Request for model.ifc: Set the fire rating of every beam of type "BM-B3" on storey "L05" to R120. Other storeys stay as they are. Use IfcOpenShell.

First a look at what the model holds.

```python
import ifcopenshell
import ifcopenshell.util.element

model = ifcopenshell.open("model.ifc")
print(model.schema)
storey = next(s for s in model.by_type("IfcBuildingStorey") if s.Name == "L05")
beams = [e for e in ifcopenshell.util.element.get_decomposition(storey) if e.is_a("IfcBeam")]
seen = {}
for e in beams:
    element_type = ifcopenshell.util.element.get_type(e)
    key = (element_type.Name if element_type != e and element_type else None, ifcopenshell.util.element.get_pset(e, "Pset_BeamCommon", "FireRating"))
    seen[key] = seen.get(key, 0) + 1
for (name, value), count in sorted(seen.items(), key=str):
    print(count, "x", name, "|", value)
```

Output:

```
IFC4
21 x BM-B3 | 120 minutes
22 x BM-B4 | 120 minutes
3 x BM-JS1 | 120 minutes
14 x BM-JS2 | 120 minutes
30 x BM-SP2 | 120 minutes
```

```python
import ifcopenshell
import ifcopenshell.api.pset
import ifcopenshell.util.element

model = ifcopenshell.open("model.ifc")

storey = next(s for s in model.by_type("IfcBuildingStorey") if s.Name == "L05")
beams = [e for e in ifcopenshell.util.element.get_decomposition(storey) if e.is_a("IfcBeam")]

count = 0
for e in beams:
    element_type = ifcopenshell.util.element.get_type(e)
    if element_type in (None, e) or element_type.Name != "BM-B3":
        continue
    # add_pset returns the element's existing set when there is one.
    pset = ifcopenshell.api.pset.add_pset(model, product=e, name="Pset_BeamCommon")
    ifcopenshell.api.pset.edit_pset(model, pset=pset, properties={"FireRating": "R120"})
    count += 1

print(count, "beams updated")

model.write("model_v2.ifc")
```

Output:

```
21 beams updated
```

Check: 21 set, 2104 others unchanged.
